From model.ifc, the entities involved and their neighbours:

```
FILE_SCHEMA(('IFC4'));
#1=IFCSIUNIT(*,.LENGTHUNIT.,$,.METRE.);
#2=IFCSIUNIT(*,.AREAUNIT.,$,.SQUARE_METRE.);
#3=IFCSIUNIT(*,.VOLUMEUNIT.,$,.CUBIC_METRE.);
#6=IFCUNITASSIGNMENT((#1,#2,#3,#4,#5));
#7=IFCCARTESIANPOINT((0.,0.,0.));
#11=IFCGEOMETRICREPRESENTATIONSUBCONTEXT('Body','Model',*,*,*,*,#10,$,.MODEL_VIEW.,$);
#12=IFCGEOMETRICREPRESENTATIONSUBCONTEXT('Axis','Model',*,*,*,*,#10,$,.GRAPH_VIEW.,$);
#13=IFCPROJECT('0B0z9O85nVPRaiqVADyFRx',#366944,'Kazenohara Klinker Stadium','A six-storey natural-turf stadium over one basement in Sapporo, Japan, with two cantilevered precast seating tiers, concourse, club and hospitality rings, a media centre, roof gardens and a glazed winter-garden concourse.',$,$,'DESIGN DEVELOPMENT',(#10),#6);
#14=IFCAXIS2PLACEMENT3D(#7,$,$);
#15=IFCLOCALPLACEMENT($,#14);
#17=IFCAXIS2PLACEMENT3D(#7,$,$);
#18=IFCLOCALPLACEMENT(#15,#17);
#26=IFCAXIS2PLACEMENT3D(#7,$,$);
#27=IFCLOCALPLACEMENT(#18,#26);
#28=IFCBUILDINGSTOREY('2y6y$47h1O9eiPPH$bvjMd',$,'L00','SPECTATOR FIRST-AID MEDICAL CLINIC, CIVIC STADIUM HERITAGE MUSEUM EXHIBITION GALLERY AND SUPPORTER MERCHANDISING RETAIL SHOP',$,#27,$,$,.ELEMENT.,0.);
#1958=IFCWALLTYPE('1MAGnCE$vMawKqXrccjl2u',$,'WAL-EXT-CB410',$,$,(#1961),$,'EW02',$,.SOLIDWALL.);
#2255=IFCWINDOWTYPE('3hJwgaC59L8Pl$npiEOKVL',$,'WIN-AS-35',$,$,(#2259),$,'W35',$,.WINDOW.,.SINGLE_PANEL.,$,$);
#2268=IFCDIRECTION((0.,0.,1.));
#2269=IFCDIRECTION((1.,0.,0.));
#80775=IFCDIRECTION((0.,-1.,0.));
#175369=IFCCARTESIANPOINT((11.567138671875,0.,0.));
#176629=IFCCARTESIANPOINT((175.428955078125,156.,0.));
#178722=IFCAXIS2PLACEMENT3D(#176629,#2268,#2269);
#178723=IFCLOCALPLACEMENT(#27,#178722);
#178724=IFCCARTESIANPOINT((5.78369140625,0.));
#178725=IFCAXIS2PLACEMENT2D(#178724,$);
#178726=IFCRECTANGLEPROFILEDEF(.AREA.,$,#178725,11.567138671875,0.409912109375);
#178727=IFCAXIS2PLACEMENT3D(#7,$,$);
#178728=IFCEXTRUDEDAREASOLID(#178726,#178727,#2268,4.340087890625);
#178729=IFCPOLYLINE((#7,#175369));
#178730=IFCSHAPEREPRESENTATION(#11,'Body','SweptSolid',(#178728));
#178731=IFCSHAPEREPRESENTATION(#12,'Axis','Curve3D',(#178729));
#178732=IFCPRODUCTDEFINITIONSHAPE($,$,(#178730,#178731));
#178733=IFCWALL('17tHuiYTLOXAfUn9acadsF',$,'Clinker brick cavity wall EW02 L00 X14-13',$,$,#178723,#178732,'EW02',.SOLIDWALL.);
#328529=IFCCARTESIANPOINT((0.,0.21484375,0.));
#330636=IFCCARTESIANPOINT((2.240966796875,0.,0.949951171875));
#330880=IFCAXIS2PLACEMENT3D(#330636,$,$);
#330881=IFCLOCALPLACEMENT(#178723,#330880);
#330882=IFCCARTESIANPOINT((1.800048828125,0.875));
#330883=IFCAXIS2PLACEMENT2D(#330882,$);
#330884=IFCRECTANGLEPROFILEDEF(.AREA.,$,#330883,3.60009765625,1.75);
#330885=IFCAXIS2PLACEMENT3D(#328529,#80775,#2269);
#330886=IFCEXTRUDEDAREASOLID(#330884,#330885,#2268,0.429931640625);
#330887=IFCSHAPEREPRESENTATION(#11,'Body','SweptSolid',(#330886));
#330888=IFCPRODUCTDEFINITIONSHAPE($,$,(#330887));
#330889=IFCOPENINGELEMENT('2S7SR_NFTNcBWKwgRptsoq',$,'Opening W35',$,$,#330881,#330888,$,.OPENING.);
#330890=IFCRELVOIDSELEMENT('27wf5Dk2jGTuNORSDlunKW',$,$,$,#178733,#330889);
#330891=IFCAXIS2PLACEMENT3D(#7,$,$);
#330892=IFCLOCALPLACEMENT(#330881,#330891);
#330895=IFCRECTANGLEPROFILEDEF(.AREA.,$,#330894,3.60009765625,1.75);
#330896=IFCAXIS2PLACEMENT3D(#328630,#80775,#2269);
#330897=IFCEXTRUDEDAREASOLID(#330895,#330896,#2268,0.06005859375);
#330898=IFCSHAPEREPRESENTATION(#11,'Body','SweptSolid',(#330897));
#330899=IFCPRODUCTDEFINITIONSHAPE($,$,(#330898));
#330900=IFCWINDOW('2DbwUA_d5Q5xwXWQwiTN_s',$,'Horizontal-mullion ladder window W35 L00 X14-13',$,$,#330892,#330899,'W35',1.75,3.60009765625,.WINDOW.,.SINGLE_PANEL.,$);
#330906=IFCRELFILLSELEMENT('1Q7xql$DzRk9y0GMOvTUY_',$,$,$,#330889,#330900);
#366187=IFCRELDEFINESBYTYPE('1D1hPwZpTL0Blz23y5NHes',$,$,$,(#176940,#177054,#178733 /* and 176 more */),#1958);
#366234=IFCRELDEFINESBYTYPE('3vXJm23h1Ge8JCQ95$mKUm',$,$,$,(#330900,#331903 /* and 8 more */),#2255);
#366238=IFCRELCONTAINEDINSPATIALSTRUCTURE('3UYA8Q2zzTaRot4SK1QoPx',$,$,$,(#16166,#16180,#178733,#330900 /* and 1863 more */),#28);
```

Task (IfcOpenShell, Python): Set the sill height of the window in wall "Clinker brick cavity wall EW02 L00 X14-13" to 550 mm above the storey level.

```python
import numpy as np
import ifcopenshell
import ifcopenshell.api.geometry
import ifcopenshell.geom
import ifcopenshell.util.element
import ifcopenshell.util.placement
import ifcopenshell.util.shape
import ifcopenshell.util.unit

model = ifcopenshell.open("model.ifc")
unit_scale = ifcopenshell.util.unit.calculate_unit_scale(model)

window = model.by_id(330900)
opening = window.FillsVoids[0].RelatingOpeningElement
storey = ifcopenshell.util.element.get_container(window, ifc_class="IfcBuildingStorey")
level = ifcopenshell.util.placement.get_local_placement(storey.ObjectPlacement)[2, 3]

# The opening's origin need not be at the sill, so measure its lowest point.
shape = ifcopenshell.geom.create_shape(ifcopenshell.geom.settings(), opening)
bottom = ifcopenshell.util.shape.get_shape_bottom_elevation(shape, shape.geometry) / unit_scale
dz = level + 0.55 / unit_scale - bottom

shift = np.array([0.0, 0.0, dz])
# The window is placed relative to its opening, so it follows when the opening moves.
matrix = ifcopenshell.util.placement.get_local_placement(opening.ObjectPlacement)
matrix[:3, 3] += shift
ifcopenshell.api.geometry.edit_object_placement(
    model, product=opening, matrix=matrix, is_si=False, should_transform_children=True
)

print(f"moved by {dz * unit_scale:+.3f} m")

model.write("model_v2.ifc")
```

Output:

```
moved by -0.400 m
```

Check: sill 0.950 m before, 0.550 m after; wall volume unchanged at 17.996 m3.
